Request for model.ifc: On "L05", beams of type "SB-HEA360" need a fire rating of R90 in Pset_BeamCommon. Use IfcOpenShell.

First a look at what the model holds.

```python
import ifcopenshell
import ifcopenshell.util.element

model = ifcopenshell.open("model.ifc")
print(model.schema)
storey = next(s for s in model.by_type("IfcBuildingStorey") if s.Name == "L05")
beams = [e for e in ifcopenshell.util.element.get_decomposition(storey) if e.is_a("IfcBeam")]
seen = {}
for e in beams:
    element_type = ifcopenshell.util.element.get_type(e)
    key = (element_type.Name if element_type != e and element_type else None, ifcopenshell.util.element.get_pset(e, "Pset_BeamCommon", "FireRating"))
    seen[key] = seen.get(key, 0) + 1
for (name, value), count in sorted(seen.items(), key=str):
    print(count, "x", name, "|", value)
```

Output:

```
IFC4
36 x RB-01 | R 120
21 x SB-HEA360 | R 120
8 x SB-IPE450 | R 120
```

```python
import ifcopenshell
import ifcopenshell.api.pset
import ifcopenshell.util.element

model = ifcopenshell.open("model.ifc")

storey = next(s for s in model.by_type("IfcBuildingStorey") if s.Name == "L05")
beams = [e for e in ifcopenshell.util.element.get_decomposition(storey) if e.is_a("IfcBeam")]

count = 0
for e in beams:
    element_type = ifcopenshell.util.element.get_type(e)
    if element_type in (None, e) or element_type.Name != "SB-HEA360":
        continue
    # add_pset returns the element's existing set when there is one.
    pset = ifcopenshell.api.pset.add_pset(model, product=e, name="Pset_BeamCommon")
    ifcopenshell.api.pset.edit_pset(model, pset=pset, properties={"FireRating": "R90"})
    count += 1

print(count, "beams updated")

model.write("model_rev.ifc")
```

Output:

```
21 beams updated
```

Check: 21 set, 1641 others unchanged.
